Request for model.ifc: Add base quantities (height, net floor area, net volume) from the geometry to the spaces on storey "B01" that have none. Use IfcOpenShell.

First a look at what the model holds.

```python
import ifcopenshell
import ifcopenshell.util.element
import ifcopenshell.util.unit

model = ifcopenshell.open("model.ifc")
print(model.schema)
for unit_type in ("LENGTHUNIT", "AREAUNIT", "VOLUMEUNIT"):
    print(unit_type, ifcopenshell.util.unit.calculate_unit_scale(model, unit_type))
storey = next(s for s in model.by_type("IfcBuildingStorey") if s.Name == "B01")
spaces = [e for e in ifcopenshell.util.element.get_decomposition(storey) if e.is_a("IfcSpace")]
for e in sorted(spaces, key=lambda e: e.id()):
    print(e.id(), e.is_a(), e.Name, list(ifcopenshell.util.element.get_psets(e, qtos_only=True)), sep=" | ")
```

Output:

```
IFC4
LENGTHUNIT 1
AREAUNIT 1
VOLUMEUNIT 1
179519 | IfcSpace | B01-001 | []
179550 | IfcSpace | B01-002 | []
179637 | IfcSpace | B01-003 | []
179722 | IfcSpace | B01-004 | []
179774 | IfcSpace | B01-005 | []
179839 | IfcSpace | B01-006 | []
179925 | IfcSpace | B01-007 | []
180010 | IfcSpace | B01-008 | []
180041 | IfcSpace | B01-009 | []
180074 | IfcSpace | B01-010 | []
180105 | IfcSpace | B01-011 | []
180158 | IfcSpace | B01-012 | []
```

```python
import ifcopenshell
import ifcopenshell.api.pset
import ifcopenshell.geom
import ifcopenshell.util.element
import ifcopenshell.util.shape
import ifcopenshell.util.unit

model = ifcopenshell.open("model.ifc")
unit_scale = ifcopenshell.util.unit.calculate_unit_scale(model)
area_scale = ifcopenshell.util.unit.calculate_unit_scale(model, "AREAUNIT")
volume_scale = ifcopenshell.util.unit.calculate_unit_scale(model, "VOLUMEUNIT")
settings = ifcopenshell.geom.settings()

storey = next(s for s in model.by_type("IfcBuildingStorey") if s.Name == "B01")
spaces = [e for e in ifcopenshell.util.element.get_decomposition(storey) if e.is_a("IfcSpace")]

for e in sorted(spaces, key=lambda e: e.id()):
    if ifcopenshell.util.element.get_psets(e, qtos_only=True, should_inherit=False):
        continue
    # Geometry comes back in metres, in the element's own axes.
    shape = ifcopenshell.geom.create_shape(settings, e)
    values = {
        "Height": ifcopenshell.util.shape.get_z(shape.geometry) / unit_scale,
        "NetFloorArea": ifcopenshell.util.shape.get_footprint_area(shape.geometry) / area_scale,
        "NetVolume": ifcopenshell.util.shape.get_volume(shape.geometry) / volume_scale,
    }
    qto = ifcopenshell.api.pset.add_qto(model, product=e, name="Qto_SpaceBaseQuantities")
    ifcopenshell.api.pset.edit_qto(model, qto=qto, properties=values)
    print(e.id(), {k: round(v, 3) for k, v in values.items()})

model.write("model-out.ifc")
```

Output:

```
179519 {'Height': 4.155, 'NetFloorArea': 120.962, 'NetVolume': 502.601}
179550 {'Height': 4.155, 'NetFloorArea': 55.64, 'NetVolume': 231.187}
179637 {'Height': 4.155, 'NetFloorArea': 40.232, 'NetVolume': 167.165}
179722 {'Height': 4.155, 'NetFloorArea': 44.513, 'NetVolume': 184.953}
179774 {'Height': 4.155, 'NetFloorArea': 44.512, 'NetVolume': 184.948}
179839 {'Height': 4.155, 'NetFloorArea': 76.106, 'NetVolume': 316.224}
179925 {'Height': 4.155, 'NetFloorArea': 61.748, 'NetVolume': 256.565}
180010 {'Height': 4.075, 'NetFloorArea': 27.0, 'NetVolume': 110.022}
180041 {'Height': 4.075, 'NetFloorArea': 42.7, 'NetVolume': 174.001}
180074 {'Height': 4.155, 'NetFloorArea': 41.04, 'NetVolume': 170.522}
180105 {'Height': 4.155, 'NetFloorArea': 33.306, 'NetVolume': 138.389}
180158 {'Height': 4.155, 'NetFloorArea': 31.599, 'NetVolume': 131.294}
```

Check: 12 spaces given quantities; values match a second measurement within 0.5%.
